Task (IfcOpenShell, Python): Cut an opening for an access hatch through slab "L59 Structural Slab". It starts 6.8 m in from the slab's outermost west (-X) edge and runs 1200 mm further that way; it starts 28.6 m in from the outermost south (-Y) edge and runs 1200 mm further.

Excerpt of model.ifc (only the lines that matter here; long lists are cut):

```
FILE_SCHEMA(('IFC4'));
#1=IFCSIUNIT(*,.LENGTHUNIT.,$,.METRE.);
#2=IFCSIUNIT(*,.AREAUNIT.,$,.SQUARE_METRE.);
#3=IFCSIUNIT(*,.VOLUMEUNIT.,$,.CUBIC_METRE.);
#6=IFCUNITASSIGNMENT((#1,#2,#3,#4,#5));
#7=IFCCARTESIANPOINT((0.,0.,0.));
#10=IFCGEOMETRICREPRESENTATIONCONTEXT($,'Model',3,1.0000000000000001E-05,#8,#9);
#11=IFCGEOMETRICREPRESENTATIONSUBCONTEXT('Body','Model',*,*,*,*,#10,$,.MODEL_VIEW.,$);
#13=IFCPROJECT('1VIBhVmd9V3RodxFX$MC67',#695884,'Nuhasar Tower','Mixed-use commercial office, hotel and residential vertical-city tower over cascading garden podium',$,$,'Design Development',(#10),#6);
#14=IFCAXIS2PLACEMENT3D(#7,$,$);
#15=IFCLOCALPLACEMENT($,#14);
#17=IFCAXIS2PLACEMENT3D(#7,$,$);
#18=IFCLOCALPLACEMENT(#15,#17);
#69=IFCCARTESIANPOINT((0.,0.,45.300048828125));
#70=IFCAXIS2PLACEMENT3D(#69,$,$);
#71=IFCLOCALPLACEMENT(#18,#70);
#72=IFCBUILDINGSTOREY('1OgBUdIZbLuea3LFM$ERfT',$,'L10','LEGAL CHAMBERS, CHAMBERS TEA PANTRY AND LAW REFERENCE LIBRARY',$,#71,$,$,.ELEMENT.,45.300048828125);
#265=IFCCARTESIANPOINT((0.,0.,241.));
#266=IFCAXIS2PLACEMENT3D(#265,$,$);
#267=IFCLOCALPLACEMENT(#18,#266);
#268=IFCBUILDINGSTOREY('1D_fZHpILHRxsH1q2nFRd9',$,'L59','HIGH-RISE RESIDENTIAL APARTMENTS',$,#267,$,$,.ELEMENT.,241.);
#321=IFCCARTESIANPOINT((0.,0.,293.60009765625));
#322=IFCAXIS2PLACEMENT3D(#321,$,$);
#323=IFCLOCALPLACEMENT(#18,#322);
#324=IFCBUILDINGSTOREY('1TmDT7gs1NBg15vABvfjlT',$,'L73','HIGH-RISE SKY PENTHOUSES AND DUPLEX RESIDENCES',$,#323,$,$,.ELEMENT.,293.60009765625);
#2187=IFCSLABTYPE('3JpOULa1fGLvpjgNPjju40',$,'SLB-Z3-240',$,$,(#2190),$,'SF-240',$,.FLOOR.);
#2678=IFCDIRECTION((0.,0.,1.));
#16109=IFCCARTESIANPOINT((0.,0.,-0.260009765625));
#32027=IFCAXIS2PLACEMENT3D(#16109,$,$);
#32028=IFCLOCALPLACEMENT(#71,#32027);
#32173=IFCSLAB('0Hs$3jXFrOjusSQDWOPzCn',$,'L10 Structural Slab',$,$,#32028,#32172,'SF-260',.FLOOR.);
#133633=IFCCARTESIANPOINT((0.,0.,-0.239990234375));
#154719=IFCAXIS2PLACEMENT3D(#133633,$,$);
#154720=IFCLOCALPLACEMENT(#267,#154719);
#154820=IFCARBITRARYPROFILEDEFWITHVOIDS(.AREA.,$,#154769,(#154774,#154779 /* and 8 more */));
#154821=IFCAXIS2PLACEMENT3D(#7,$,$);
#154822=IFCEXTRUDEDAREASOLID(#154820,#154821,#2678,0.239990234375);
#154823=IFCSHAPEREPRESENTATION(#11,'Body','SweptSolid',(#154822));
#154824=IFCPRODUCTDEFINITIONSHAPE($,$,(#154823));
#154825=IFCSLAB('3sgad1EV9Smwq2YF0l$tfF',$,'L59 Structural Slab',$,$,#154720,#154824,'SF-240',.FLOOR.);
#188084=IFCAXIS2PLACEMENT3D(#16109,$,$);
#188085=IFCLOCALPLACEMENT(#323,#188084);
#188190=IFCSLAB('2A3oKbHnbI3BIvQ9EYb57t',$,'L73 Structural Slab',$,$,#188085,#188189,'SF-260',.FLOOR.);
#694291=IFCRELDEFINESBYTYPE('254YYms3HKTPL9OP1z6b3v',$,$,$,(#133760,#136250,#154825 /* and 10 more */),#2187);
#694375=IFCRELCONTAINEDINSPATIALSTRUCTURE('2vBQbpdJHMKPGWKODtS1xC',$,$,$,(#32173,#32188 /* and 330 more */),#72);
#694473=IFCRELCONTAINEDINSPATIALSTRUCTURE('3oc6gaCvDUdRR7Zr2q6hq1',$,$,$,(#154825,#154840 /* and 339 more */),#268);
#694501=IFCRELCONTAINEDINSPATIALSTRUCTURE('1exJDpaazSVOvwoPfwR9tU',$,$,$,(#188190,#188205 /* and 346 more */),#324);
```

```python
import numpy as np
import ifcopenshell
import ifcopenshell.api.feature
import ifcopenshell.api.geometry
import ifcopenshell.api.root
import ifcopenshell.geom
import ifcopenshell.util.placement
import ifcopenshell.util.representation
import ifcopenshell.util.shape
import ifcopenshell.util.unit

model = ifcopenshell.open("model.ifc")
unit_scale = ifcopenshell.util.unit.calculate_unit_scale(model)
settings = ifcopenshell.geom.settings()


def volume(element):
    """Net volume in cubic metres, openings subtracted."""
    shape = ifcopenshell.geom.create_shape(settings, element)
    return ifcopenshell.util.shape.get_volume(shape.geometry)


slab = model.by_guid("3sgad1EV9Smwq2YF0l$tfF")
before = volume(slab)

# Extent in the slab's own axes, in metres. The edges named are its -X and -Y sides.
slab_shape = ifcopenshell.geom.create_shape(settings, slab)
vertices = ifcopenshell.util.shape.get_vertices(slab_shape.geometry)
x_min, y_min, bottom = vertices.min(axis=0)
top = vertices[:, 2].max()

opening = ifcopenshell.api.root.create_entity(model, ifc_class="IfcOpeningElement", name="Access hatch opening", predefined_type="OPENING")
context = ifcopenshell.util.representation.get_context(model, "Model", "Body", "MODEL_VIEW")
width, depth = 1.2, 1.2
outline = [(0.0, 0.0), (width, 0.0), (width, depth), (0.0, depth), (0.0, 0.0)]
# Overshoot both faces by 50 mm so the cut is clean.
shape = ifcopenshell.api.geometry.add_slab_representation(
    model, context=context, depth=top - bottom + 0.1, polyline=outline
)
ifcopenshell.api.geometry.assign_representation(model, product=opening, representation=shape)

matrix = ifcopenshell.util.placement.get_local_placement(slab.ObjectPlacement)
matrix[:, 3] = matrix @ np.append(np.array([x_min + 6.8, y_min + 28.6, bottom - 0.05]) / unit_scale, 1.0)
ifcopenshell.api.geometry.edit_object_placement(model, product=opening, matrix=matrix, is_si=False)
ifcopenshell.api.feature.add_feature(model, feature=opening, element=slab)

after = volume(slab)

print(f"slab volume {before:.3f} -> {after:.3f} m3")

model.write("model_updated.ifc")
```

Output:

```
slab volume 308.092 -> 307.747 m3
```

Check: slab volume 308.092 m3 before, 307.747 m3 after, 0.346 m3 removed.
